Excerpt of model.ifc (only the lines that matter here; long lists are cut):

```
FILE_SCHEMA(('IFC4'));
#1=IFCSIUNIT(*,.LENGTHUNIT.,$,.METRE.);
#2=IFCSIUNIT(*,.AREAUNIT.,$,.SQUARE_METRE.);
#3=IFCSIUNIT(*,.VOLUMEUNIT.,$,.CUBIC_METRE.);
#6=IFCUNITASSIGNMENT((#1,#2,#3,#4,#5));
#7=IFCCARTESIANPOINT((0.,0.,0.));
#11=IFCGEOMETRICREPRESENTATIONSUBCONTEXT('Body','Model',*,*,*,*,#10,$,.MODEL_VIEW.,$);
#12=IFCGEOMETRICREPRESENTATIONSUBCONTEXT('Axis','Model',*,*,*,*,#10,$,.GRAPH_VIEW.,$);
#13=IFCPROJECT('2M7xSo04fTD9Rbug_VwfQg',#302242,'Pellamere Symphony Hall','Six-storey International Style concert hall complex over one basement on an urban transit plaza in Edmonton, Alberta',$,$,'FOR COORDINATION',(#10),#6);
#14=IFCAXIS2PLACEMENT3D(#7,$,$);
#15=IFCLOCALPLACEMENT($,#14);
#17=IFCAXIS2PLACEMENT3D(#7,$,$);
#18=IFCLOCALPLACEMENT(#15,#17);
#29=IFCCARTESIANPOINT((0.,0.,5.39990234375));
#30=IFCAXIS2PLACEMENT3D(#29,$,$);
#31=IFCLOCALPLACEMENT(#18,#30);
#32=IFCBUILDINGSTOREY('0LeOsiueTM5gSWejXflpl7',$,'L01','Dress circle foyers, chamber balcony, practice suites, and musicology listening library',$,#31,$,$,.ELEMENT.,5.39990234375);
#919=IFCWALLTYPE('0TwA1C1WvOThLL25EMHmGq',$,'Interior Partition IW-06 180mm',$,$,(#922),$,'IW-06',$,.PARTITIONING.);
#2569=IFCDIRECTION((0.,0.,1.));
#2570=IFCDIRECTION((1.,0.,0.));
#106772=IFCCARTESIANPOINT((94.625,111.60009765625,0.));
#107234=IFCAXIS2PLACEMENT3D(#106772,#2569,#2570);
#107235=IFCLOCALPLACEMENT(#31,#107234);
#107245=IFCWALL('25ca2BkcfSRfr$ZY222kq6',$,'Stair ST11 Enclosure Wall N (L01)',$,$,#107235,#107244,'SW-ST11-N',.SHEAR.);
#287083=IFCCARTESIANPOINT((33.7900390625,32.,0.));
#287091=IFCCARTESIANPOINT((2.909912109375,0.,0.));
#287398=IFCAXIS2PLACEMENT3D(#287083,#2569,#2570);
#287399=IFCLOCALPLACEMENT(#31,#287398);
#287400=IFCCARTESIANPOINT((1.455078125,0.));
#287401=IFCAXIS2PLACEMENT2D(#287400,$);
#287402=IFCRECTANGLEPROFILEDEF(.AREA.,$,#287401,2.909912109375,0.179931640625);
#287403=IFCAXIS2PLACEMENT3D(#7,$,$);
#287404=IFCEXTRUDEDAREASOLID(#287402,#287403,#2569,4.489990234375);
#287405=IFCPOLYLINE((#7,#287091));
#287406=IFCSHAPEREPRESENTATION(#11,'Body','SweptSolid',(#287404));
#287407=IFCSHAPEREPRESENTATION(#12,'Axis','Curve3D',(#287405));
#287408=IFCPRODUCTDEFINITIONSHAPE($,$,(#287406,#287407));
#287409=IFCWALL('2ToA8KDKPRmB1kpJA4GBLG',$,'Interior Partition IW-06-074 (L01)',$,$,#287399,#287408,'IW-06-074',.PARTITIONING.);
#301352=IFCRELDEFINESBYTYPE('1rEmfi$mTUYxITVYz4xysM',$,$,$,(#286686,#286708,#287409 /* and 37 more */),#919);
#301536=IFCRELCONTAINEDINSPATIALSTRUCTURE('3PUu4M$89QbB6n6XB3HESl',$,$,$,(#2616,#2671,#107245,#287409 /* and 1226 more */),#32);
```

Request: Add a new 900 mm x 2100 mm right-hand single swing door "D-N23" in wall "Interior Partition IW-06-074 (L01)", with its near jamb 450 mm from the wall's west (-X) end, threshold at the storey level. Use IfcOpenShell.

```python
import numpy as np
import ifcopenshell
import ifcopenshell.api.feature
import ifcopenshell.api.geometry
import ifcopenshell.api.root
import ifcopenshell.api.spatial
import ifcopenshell.geom
import ifcopenshell.util.element
import ifcopenshell.util.placement
import ifcopenshell.util.representation
import ifcopenshell.util.shape
import ifcopenshell.util.unit

model = ifcopenshell.open("model.ifc")
unit_scale = ifcopenshell.util.unit.calculate_unit_scale(model)
settings = ifcopenshell.geom.settings()


def volume(element):
    """Net volume in cubic metres, openings subtracted."""
    shape = ifcopenshell.geom.create_shape(settings, element)
    return ifcopenshell.util.shape.get_volume(shape.geometry)


wall = model.by_id(287409)
storey = ifcopenshell.util.element.get_container(wall, ifc_class="IfcBuildingStorey")
context = ifcopenshell.util.representation.get_context(model, "Model", "Body", "MODEL_VIEW")
before = volume(wall)

width, height, from_end, sill = 0.9, 2.1, 0.45, 0.0  # metres

# The wall runs along its own X axis, and the end named is its -X end.
wall_shape = ifcopenshell.geom.create_shape(settings, wall)
x, y, z = ifcopenshell.util.shape.get_vertices(wall_shape.geometry).T
start = x.min() + from_end
face, thickness = float(y.min()), float(y.max() - y.min())
wall_matrix = ifcopenshell.util.placement.get_local_placement(wall.ObjectPlacement)
level = ifcopenshell.util.placement.get_local_placement(storey.ObjectPlacement)[2, 3]


def in_wall(x, y):
    """Placement at x, y metres in the wall's axes, at sill height."""
    matrix = wall_matrix.copy()
    matrix[:, 3] = wall_matrix @ np.array([x / unit_scale, y / unit_scale, 0.0, 1.0])
    matrix[2, 3] = level + sill / unit_scale
    return matrix


# Opening: a box that overshoots both wall faces by 50 mm.
opening = ifcopenshell.api.root.create_entity(model, ifc_class="IfcOpeningElement", predefined_type="OPENING")
box = ifcopenshell.api.geometry.add_wall_representation(
    model, context=context, length=width, height=height, thickness=thickness + 0.1
)
ifcopenshell.api.geometry.assign_representation(model, product=opening, representation=box)
ifcopenshell.api.geometry.edit_object_placement(model, product=opening, matrix=in_wall(start, face - 0.05), is_si=False)
ifcopenshell.api.feature.add_feature(model, feature=opening, element=wall)

door = ifcopenshell.api.root.create_entity(model, ifc_class="IfcDoor", name="D-N23", predefined_type="DOOR")
door.OverallWidth, door.OverallHeight = width / unit_scale, height / unit_scale
door.OperationType = "SINGLE_SWING_RIGHT"
body = ifcopenshell.api.geometry.add_door_representation(
    model,
    context=context,
    overall_width=door.OverallWidth,
    overall_height=door.OverallHeight,
    operation_type="SINGLE_SWING_RIGHT",
    lining_properties={"LiningDepth": thickness / unit_scale, "ThresholdDepth": thickness / unit_scale},
)
ifcopenshell.api.geometry.assign_representation(model, product=door, representation=body)
ifcopenshell.api.spatial.assign_container(model, products=[door], relating_structure=storey)
ifcopenshell.api.feature.add_filling(model, opening=opening, element=door)

# The lining spans the wall, so the door starts at the wall face.
ifcopenshell.api.geometry.edit_object_placement(model, product=door, matrix=in_wall(start, face), is_si=False)

after = volume(wall)

print(f"wall volume {before:.3f} -> {after:.3f} m3")

model.write("model-out.ifc")
```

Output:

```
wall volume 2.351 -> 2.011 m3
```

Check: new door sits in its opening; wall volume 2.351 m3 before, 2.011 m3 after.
